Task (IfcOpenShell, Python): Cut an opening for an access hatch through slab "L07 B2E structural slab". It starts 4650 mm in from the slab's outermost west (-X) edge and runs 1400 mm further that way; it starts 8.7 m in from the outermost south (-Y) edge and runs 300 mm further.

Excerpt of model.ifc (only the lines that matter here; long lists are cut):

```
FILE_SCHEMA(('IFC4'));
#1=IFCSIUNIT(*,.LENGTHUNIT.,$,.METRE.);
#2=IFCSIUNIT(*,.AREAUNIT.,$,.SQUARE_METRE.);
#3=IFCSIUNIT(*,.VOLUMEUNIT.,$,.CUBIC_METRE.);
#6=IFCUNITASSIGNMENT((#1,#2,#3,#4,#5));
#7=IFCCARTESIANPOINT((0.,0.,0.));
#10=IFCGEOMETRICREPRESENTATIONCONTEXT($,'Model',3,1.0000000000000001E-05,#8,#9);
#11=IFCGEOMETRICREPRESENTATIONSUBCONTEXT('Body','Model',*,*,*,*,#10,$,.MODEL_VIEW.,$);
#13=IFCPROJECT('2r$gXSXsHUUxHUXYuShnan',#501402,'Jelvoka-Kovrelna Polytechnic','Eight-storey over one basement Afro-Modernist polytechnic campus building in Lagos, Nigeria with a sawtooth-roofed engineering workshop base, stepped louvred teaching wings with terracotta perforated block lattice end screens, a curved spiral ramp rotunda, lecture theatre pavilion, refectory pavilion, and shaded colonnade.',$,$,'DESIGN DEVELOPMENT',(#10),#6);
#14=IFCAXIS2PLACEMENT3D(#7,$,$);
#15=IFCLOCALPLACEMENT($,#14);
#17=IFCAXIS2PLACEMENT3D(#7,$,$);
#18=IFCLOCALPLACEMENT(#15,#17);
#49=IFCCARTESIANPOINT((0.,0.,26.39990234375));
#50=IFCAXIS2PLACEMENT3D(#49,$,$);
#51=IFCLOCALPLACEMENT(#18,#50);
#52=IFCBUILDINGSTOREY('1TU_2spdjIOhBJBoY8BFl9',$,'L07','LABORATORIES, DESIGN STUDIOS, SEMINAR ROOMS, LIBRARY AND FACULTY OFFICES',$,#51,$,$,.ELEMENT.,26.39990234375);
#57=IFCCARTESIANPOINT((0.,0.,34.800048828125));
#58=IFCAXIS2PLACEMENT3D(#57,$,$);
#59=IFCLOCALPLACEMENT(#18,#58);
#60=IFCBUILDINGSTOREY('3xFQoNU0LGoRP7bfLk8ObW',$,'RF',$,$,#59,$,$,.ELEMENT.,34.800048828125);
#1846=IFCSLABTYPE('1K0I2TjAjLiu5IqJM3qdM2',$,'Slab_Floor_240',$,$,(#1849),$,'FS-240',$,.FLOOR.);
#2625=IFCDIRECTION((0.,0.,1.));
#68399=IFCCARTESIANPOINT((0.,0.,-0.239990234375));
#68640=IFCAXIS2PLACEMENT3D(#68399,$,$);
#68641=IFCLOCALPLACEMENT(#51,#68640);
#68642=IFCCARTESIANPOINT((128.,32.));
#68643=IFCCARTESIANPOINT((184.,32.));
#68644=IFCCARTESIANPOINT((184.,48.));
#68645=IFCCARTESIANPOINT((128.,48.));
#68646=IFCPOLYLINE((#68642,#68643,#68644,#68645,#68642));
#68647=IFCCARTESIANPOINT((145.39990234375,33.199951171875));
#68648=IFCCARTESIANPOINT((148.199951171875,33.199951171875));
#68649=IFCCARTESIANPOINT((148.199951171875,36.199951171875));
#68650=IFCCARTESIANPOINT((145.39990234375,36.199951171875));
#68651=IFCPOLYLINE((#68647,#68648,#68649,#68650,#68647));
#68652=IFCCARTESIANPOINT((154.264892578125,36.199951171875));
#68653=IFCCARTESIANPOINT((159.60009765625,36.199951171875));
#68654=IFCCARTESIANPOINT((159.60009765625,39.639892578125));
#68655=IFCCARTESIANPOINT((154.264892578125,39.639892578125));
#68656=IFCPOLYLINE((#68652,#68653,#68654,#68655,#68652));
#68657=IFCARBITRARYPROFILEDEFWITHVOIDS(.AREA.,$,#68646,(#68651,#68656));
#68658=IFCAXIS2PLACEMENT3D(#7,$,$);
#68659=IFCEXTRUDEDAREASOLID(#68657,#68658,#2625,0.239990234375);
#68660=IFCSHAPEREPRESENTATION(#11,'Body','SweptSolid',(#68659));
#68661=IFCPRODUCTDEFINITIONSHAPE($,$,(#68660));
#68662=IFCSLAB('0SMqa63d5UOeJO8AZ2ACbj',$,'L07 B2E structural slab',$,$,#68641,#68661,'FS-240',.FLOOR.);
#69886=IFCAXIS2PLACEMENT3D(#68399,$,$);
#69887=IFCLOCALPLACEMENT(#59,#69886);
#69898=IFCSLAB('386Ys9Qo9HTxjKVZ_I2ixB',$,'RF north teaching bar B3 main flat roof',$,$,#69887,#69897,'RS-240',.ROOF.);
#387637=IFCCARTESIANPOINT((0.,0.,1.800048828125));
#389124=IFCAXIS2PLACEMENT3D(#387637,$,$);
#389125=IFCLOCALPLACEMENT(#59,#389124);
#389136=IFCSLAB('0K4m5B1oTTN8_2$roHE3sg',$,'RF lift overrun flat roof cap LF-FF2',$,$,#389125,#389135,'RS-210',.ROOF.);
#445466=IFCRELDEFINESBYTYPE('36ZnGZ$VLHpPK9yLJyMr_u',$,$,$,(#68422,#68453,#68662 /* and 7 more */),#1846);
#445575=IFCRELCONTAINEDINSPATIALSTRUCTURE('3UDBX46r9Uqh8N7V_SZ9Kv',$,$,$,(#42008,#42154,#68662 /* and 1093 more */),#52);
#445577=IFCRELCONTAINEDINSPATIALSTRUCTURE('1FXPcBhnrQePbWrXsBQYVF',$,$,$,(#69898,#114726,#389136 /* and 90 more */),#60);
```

```python
import numpy as np
import ifcopenshell
import ifcopenshell.api.feature
import ifcopenshell.api.geometry
import ifcopenshell.api.root
import ifcopenshell.geom
import ifcopenshell.util.placement
import ifcopenshell.util.representation
import ifcopenshell.util.shape
import ifcopenshell.util.unit

model = ifcopenshell.open("model.ifc")
unit_scale = ifcopenshell.util.unit.calculate_unit_scale(model)
settings = ifcopenshell.geom.settings()


def volume(element):
    """Net volume in cubic metres, openings subtracted."""
    shape = ifcopenshell.geom.create_shape(settings, element)
    return ifcopenshell.util.shape.get_volume(shape.geometry)


slab = model.by_id(68662)
before = volume(slab)

# Extent in the slab's own axes, in metres. The edges named are its -X and -Y sides.
slab_shape = ifcopenshell.geom.create_shape(settings, slab)
vertices = ifcopenshell.util.shape.get_vertices(slab_shape.geometry)
x_min, y_min, bottom = vertices.min(axis=0)
top = vertices[:, 2].max()

opening = ifcopenshell.api.root.create_entity(model, ifc_class="IfcOpeningElement", name="Access hatch opening", predefined_type="OPENING")
context = ifcopenshell.util.representation.get_context(model, "Model", "Body", "MODEL_VIEW")
width, depth = 1.4, 0.3
outline = [(0.0, 0.0), (width, 0.0), (width, depth), (0.0, depth), (0.0, 0.0)]
# Overshoot both faces by 50 mm so the cut is clean.
shape = ifcopenshell.api.geometry.add_slab_representation(
    model, context=context, depth=top - bottom + 0.1, polyline=outline
)
ifcopenshell.api.geometry.assign_representation(model, product=opening, representation=shape)

matrix = ifcopenshell.util.placement.get_local_placement(slab.ObjectPlacement)
matrix[:, 3] = matrix @ np.append(np.array([x_min + 4.65, y_min + 8.7, bottom - 0.05]) / unit_scale, 1.0)
ifcopenshell.api.geometry.edit_object_placement(model, product=opening, matrix=matrix, is_si=False)
ifcopenshell.api.feature.add_feature(model, feature=opening, element=slab)

after = volume(slab)

print(f"slab volume {before:.3f} -> {after:.3f} m3")

model.write("model-out.ifc")
```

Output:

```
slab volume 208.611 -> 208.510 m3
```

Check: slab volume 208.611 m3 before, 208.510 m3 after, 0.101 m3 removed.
